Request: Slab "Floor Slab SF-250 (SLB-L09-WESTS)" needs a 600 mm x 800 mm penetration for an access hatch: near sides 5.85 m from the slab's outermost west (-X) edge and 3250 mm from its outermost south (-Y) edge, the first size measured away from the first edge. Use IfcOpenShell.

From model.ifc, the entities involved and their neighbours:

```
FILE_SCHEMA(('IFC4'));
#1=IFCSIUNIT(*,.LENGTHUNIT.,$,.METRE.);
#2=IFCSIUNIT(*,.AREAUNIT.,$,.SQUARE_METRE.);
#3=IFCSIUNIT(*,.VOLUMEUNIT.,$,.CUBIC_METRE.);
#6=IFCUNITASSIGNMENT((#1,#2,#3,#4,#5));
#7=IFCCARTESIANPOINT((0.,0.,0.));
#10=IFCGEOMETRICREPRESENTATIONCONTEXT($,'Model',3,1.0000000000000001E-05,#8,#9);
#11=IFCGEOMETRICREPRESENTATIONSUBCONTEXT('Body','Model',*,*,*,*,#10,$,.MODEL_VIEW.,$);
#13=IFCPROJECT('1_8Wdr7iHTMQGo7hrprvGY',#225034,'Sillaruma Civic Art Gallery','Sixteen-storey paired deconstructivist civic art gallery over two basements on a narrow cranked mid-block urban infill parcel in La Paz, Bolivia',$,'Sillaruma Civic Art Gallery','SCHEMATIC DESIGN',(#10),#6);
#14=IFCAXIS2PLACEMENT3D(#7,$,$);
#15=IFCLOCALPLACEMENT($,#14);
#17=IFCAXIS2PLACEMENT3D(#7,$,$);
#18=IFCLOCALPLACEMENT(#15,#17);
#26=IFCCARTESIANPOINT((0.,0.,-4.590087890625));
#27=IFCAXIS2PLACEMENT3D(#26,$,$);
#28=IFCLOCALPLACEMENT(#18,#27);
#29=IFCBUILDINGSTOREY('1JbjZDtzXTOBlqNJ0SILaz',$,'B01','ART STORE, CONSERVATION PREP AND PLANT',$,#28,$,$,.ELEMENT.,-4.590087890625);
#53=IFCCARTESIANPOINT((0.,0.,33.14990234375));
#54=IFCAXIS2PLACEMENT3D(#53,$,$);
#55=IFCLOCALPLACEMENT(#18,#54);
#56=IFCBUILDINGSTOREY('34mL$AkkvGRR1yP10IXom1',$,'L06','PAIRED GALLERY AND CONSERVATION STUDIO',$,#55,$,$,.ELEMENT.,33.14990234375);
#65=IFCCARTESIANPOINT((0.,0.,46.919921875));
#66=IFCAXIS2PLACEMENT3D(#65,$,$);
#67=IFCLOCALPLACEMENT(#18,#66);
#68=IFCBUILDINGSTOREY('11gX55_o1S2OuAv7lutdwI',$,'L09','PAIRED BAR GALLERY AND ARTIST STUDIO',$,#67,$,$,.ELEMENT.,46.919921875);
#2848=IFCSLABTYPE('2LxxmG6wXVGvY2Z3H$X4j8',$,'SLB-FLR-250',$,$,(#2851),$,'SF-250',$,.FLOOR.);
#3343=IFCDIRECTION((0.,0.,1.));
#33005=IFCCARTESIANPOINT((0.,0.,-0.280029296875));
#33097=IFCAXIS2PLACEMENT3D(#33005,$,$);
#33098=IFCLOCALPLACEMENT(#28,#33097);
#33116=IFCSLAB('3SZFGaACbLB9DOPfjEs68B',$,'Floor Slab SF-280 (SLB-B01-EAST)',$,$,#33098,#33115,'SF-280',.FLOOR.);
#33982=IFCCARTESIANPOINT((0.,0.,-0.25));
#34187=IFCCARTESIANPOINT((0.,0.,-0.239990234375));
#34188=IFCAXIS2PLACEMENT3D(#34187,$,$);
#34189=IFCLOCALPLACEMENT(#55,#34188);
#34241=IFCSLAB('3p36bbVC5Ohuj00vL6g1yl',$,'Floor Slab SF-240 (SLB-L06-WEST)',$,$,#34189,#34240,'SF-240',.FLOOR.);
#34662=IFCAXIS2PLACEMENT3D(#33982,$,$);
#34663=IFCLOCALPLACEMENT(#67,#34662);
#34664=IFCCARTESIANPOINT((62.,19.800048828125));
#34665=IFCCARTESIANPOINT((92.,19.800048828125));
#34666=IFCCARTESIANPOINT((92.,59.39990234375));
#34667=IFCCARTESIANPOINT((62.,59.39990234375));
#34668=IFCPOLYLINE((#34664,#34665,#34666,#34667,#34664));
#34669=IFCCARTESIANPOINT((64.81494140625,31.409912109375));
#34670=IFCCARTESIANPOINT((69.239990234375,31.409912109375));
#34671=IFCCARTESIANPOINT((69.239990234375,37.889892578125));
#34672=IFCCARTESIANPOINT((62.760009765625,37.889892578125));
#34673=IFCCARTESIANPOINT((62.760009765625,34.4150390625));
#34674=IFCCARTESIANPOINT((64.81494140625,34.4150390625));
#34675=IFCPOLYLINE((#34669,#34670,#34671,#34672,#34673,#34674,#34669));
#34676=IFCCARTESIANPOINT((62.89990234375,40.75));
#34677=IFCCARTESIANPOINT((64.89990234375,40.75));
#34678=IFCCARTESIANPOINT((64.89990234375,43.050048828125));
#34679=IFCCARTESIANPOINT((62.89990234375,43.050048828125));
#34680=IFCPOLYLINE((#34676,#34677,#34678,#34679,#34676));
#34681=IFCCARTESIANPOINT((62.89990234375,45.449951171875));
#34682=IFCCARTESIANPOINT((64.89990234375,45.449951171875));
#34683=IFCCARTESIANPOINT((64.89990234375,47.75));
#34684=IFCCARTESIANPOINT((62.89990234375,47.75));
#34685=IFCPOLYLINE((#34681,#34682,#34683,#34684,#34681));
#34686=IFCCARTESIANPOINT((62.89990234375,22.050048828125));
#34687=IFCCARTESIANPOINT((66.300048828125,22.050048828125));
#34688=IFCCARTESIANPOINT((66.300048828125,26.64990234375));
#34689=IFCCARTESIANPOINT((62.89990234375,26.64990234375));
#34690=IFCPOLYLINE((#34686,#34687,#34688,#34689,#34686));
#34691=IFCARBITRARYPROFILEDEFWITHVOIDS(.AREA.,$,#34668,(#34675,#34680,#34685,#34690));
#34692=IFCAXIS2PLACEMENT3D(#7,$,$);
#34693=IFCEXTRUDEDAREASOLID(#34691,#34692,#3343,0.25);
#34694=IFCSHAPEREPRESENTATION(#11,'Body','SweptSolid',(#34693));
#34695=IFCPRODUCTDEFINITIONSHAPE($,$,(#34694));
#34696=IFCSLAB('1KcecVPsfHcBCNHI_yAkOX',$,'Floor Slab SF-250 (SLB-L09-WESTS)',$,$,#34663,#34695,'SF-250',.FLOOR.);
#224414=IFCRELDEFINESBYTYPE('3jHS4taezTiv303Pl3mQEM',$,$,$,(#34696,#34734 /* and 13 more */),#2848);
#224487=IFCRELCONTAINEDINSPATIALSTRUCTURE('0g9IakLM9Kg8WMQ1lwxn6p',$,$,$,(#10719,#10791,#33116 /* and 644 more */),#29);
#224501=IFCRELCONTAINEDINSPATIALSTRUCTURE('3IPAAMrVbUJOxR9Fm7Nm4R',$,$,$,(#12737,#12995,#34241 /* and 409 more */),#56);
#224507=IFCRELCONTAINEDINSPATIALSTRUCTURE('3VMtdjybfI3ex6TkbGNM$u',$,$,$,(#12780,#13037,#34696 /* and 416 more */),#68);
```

```python
import numpy as np
import ifcopenshell
import ifcopenshell.api.feature
import ifcopenshell.api.geometry
import ifcopenshell.api.root
import ifcopenshell.geom
import ifcopenshell.util.placement
import ifcopenshell.util.representation
import ifcopenshell.util.shape
import ifcopenshell.util.unit

model = ifcopenshell.open("model.ifc")
unit_scale = ifcopenshell.util.unit.calculate_unit_scale(model)
settings = ifcopenshell.geom.settings()


def volume(element):
    """Net volume in cubic metres, openings subtracted."""
    shape = ifcopenshell.geom.create_shape(settings, element)
    return ifcopenshell.util.shape.get_volume(shape.geometry)


slab = model.by_guid("1KcecVPsfHcBCNHI_yAkOX")
before = volume(slab)

# Extent in the slab's own axes, in metres. The edges named are its -X and -Y sides.
slab_shape = ifcopenshell.geom.create_shape(settings, slab)
vertices = ifcopenshell.util.shape.get_vertices(slab_shape.geometry)
x_min, y_min, bottom = vertices.min(axis=0)
top = vertices[:, 2].max()

opening = ifcopenshell.api.root.create_entity(model, ifc_class="IfcOpeningElement", name="Access hatch opening", predefined_type="OPENING")
context = ifcopenshell.util.representation.get_context(model, "Model", "Body", "MODEL_VIEW")
width, depth = 0.6, 0.8
outline = [(0.0, 0.0), (width, 0.0), (width, depth), (0.0, depth), (0.0, 0.0)]
# Overshoot both faces by 50 mm so the cut is clean.
shape = ifcopenshell.api.geometry.add_slab_representation(
    model, context=context, depth=top - bottom + 0.1, polyline=outline
)
ifcopenshell.api.geometry.assign_representation(model, product=opening, representation=shape)

matrix = ifcopenshell.util.placement.get_local_placement(slab.ObjectPlacement)
matrix[:, 3] = matrix @ np.append(np.array([x_min + 5.85, y_min + 3.25, bottom - 0.05]) / unit_scale, 1.0)
ifcopenshell.api.geometry.edit_object_placement(model, product=opening, matrix=matrix, is_si=False)
ifcopenshell.api.feature.add_feature(model, feature=opening, element=slab)

after = volume(slab)

print(f"slab volume {before:.3f} -> {after:.3f} m3")

model.write("model_updated.ifc")
```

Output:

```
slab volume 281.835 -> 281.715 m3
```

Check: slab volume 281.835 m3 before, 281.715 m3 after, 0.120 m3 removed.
